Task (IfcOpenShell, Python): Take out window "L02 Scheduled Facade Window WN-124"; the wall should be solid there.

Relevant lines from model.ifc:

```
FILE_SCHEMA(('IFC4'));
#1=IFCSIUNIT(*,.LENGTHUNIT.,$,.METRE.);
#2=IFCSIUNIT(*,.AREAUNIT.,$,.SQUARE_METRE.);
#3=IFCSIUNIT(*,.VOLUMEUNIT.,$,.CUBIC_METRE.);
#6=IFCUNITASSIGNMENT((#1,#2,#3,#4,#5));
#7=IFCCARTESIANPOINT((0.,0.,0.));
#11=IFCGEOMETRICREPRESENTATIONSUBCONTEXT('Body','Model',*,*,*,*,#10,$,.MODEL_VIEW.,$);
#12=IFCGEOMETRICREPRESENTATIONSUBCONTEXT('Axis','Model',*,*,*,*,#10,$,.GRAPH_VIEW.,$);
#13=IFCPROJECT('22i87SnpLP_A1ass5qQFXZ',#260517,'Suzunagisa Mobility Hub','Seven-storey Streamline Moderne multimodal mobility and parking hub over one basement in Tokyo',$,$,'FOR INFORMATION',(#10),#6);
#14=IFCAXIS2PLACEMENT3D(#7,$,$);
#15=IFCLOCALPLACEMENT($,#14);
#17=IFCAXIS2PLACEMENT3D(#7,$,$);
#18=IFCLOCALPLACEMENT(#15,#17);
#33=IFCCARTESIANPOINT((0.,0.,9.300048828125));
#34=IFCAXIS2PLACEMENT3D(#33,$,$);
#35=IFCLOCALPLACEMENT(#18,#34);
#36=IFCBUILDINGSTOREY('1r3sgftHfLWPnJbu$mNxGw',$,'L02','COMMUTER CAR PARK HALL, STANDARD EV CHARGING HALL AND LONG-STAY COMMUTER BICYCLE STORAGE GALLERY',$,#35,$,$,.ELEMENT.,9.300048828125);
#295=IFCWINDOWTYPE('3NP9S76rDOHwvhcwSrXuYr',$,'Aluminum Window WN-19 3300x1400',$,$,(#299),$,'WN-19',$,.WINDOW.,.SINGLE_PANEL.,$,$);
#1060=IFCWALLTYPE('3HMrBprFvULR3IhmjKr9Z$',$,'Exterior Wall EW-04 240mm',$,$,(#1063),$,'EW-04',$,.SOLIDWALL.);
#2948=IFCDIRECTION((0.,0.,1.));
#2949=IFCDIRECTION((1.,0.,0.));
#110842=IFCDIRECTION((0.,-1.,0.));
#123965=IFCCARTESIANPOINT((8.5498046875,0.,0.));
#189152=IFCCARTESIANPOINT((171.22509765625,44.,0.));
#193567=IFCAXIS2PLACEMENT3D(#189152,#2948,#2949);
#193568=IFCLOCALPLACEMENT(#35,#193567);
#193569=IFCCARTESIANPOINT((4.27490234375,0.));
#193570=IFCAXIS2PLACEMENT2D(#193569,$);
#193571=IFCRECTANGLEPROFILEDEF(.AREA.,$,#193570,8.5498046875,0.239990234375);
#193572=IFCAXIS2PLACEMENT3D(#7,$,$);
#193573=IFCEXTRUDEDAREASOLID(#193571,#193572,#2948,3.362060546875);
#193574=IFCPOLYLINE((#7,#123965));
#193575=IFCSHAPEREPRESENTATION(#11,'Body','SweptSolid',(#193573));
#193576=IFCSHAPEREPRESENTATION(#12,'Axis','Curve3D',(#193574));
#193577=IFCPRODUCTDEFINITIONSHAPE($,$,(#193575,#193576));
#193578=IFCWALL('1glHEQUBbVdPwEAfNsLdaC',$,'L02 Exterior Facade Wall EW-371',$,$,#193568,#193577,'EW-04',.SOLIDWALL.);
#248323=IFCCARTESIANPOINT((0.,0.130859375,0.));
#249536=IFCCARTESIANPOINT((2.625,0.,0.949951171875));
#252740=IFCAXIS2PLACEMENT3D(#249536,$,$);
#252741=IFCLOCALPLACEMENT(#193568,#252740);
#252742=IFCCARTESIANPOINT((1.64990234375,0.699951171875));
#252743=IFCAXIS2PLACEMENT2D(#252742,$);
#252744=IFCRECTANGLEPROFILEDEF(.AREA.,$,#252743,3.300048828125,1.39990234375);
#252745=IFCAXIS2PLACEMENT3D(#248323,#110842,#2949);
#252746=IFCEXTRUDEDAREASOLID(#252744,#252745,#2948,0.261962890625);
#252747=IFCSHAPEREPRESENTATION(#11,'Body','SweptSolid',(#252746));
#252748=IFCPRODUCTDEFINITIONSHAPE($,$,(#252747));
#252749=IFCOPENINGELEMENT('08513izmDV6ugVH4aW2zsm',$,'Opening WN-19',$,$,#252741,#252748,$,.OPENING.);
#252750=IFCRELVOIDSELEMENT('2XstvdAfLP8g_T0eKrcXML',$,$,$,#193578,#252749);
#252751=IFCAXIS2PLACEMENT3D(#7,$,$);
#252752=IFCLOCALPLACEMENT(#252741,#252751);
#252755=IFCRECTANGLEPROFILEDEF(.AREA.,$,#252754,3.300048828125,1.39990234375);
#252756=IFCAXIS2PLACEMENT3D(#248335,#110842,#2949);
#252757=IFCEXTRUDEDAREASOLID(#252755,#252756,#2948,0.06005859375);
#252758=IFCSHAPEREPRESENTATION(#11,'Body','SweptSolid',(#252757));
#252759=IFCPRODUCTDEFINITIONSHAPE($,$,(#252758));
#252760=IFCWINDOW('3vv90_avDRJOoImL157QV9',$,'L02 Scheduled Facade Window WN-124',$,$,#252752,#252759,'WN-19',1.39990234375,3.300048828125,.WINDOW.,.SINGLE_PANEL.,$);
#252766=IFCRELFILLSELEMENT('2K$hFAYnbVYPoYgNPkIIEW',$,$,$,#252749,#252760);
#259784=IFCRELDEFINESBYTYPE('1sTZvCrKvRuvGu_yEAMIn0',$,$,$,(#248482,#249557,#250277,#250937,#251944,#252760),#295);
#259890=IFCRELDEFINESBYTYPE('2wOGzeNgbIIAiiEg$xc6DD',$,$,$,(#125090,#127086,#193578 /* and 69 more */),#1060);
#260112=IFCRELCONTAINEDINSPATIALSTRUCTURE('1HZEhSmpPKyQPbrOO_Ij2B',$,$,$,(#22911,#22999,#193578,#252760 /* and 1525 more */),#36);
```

```python
import ifcopenshell
import ifcopenshell.api.feature
import ifcopenshell.api.root
import ifcopenshell.geom
import ifcopenshell.util.shape

model = ifcopenshell.open("model.ifc")
settings = ifcopenshell.geom.settings()


def volume(element):
    """Net volume in cubic metres, openings subtracted."""
    shape = ifcopenshell.geom.create_shape(settings, element)
    return ifcopenshell.util.shape.get_volume(shape.geometry)


window = model.by_guid("3vv90_avDRJOoImL157QV9")
opening = window.FillsVoids[0].RelatingOpeningElement
wall = opening.VoidsElements[0].RelatingBuildingElement
before = volume(wall)

ifcopenshell.api.root.remove_product(model, product=window)
ifcopenshell.api.feature.remove_feature(model, feature=opening)

after = volume(wall)

print(f"wall volume {before:.3f} -> {after:.3f} m3")

model.write("model-out.ifc")
```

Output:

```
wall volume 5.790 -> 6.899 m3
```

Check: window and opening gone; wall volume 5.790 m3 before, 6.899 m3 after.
